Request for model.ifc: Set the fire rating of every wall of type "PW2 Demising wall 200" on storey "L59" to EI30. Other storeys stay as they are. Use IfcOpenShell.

First a look at what the model holds.

```python
import ifcopenshell
import ifcopenshell.util.element

model = ifcopenshell.open("model.ifc")
print(model.schema)
storey = next(s for s in model.by_type("IfcBuildingStorey") if s.Name == "L59")
walls = [e for e in ifcopenshell.util.element.get_decomposition(storey) if e.is_a("IfcWall")]
seen = {}
for e in walls:
    element_type = ifcopenshell.util.element.get_type(e)
    key = (element_type.Name if element_type != e and element_type else None, ifcopenshell.util.element.get_pset(e, "Pset_WallCommon", "FireRating"))
    seen[key] = seen.get(key, 0) + 1
for (name, value), count in sorted(seen.items(), key=str):
    print(count, "x", name, "|", value)
```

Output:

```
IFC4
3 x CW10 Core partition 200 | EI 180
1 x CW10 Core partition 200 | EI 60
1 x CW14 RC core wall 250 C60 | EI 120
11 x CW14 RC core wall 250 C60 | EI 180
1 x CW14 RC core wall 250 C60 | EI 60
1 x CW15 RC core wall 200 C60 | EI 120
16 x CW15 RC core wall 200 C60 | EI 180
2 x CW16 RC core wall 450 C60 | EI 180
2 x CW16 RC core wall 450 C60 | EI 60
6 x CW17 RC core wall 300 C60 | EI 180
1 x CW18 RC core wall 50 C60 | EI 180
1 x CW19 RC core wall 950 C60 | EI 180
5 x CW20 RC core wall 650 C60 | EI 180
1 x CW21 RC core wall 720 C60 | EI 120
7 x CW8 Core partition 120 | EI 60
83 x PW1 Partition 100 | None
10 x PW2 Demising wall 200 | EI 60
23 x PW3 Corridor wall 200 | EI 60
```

```python
import ifcopenshell
import ifcopenshell.api.pset
import ifcopenshell.util.element

model = ifcopenshell.open("model.ifc")

storey = next(s for s in model.by_type("IfcBuildingStorey") if s.Name == "L59")
walls = [e for e in ifcopenshell.util.element.get_decomposition(storey) if e.is_a("IfcWall")]

count = 0
for e in walls:
    element_type = ifcopenshell.util.element.get_type(e)
    if element_type in (None, e) or element_type.Name != "PW2 Demising wall 200":
        continue
    found = ifcopenshell.util.element.get_pset(e, "Pset_WallCommon", should_inherit=False)
    if found:
        pset = model.by_id(found["id"])
        if len(ifcopenshell.util.element.get_elements_by_pset(pset)) > 1:
            pset = ifcopenshell.api.pset.unshare_pset(model, products=[e], pset=pset)[0]
    else:
        pset = ifcopenshell.api.pset.add_pset(model, product=e, name="Pset_WallCommon")
    ifcopenshell.api.pset.edit_pset(model, pset=pset, properties={"FireRating": "EI30"})
    count += 1

print(count, "walls updated")

model.write("model_rev.ifc")
```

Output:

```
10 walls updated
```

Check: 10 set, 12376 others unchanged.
